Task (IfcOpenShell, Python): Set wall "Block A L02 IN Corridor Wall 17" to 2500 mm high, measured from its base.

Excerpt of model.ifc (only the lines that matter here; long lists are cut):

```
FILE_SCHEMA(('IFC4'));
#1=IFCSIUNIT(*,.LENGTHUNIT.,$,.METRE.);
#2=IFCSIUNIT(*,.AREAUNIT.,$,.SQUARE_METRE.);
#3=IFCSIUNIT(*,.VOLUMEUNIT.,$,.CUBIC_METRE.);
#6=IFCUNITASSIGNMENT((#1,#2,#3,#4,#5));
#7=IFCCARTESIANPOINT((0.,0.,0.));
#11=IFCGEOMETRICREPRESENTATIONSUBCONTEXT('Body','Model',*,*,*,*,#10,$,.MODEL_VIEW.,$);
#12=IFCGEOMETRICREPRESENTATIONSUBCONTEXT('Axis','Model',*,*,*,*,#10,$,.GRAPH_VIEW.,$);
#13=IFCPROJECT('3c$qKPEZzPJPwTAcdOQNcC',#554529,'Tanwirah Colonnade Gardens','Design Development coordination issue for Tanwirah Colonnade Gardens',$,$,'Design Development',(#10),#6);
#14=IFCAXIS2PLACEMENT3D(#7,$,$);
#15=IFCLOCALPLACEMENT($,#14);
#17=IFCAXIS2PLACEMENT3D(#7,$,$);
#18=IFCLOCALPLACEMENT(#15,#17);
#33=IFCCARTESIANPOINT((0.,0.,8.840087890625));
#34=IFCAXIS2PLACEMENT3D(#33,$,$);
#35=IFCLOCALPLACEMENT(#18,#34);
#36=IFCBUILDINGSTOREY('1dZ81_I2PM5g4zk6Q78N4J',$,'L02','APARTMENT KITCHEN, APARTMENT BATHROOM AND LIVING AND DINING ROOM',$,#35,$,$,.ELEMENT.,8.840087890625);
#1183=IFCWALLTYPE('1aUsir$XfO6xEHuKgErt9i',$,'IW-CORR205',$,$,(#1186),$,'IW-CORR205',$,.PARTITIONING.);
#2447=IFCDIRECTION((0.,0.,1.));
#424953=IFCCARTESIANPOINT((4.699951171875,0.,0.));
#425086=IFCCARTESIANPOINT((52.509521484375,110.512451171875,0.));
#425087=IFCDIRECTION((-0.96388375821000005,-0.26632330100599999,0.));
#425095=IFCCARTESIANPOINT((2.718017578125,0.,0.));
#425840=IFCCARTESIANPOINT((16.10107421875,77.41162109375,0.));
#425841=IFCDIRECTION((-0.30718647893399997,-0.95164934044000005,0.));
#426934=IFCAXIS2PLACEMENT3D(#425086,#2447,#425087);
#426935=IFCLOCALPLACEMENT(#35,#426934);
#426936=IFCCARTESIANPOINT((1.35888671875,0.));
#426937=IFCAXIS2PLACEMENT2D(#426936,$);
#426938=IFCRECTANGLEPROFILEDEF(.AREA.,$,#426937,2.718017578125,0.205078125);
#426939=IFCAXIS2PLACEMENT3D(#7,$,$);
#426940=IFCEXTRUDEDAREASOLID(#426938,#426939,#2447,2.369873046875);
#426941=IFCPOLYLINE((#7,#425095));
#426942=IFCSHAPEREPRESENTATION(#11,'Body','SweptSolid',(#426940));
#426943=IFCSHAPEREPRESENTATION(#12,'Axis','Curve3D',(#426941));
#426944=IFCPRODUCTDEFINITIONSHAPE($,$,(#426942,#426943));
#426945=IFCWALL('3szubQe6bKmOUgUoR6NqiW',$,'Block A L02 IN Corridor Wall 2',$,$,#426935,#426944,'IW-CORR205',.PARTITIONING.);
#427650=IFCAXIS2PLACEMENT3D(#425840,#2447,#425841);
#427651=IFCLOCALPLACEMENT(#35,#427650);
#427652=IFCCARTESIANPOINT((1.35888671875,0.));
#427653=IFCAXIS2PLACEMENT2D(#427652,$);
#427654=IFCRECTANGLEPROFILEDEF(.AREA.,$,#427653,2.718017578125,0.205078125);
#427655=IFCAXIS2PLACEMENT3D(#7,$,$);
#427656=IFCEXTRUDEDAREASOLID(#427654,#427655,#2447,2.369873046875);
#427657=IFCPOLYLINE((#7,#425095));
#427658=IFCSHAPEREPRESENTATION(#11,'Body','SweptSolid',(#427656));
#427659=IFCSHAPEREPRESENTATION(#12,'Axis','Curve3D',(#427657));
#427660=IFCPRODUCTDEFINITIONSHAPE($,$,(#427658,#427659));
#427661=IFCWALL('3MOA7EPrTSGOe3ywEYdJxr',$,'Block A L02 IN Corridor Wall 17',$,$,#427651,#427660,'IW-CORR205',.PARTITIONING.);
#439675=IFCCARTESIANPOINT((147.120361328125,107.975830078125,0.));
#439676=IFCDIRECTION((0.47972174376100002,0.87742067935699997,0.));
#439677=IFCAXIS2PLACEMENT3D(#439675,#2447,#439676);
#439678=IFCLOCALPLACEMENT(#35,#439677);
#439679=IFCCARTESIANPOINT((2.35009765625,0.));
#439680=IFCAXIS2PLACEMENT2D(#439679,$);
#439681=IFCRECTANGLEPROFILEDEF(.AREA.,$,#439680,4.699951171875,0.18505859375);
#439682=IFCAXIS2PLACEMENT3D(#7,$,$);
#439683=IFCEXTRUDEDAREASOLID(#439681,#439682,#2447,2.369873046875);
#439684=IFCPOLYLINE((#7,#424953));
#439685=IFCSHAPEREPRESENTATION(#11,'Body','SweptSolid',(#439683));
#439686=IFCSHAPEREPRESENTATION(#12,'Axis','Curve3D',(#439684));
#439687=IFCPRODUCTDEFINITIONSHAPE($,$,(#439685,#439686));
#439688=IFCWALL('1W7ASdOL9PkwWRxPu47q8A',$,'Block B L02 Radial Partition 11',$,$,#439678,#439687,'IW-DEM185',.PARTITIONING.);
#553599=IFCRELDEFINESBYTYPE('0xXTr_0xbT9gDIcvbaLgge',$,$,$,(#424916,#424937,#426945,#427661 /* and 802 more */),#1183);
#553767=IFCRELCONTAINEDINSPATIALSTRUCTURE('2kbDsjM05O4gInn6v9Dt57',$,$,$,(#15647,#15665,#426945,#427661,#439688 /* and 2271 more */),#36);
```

```python
import ifcopenshell
import ifcopenshell.geom
import ifcopenshell.util.representation
import ifcopenshell.util.shape

model = ifcopenshell.open("model.ifc")
settings = ifcopenshell.geom.settings()


def volume(element):
    """Net volume in cubic metres, openings subtracted."""
    shape = ifcopenshell.geom.create_shape(settings, element)
    return ifcopenshell.util.shape.get_volume(shape.geometry)


wall = model.by_guid("3MOA7EPrTSGOe3ywEYdJxr")
before = volume(wall)

body = ifcopenshell.util.representation.get_representation(wall, "Model", "Body")
solid = body.Items[0]
old_height = solid.Depth
solid.Depth = 2.5
after = volume(wall)

print(f"height {old_height:g} -> {solid.Depth:g}, volume {before:.3f} -> {after:.3f} m3")

model.write("model-out.ifc")
```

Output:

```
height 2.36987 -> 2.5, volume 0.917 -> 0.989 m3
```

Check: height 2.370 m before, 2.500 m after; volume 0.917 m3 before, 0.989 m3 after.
